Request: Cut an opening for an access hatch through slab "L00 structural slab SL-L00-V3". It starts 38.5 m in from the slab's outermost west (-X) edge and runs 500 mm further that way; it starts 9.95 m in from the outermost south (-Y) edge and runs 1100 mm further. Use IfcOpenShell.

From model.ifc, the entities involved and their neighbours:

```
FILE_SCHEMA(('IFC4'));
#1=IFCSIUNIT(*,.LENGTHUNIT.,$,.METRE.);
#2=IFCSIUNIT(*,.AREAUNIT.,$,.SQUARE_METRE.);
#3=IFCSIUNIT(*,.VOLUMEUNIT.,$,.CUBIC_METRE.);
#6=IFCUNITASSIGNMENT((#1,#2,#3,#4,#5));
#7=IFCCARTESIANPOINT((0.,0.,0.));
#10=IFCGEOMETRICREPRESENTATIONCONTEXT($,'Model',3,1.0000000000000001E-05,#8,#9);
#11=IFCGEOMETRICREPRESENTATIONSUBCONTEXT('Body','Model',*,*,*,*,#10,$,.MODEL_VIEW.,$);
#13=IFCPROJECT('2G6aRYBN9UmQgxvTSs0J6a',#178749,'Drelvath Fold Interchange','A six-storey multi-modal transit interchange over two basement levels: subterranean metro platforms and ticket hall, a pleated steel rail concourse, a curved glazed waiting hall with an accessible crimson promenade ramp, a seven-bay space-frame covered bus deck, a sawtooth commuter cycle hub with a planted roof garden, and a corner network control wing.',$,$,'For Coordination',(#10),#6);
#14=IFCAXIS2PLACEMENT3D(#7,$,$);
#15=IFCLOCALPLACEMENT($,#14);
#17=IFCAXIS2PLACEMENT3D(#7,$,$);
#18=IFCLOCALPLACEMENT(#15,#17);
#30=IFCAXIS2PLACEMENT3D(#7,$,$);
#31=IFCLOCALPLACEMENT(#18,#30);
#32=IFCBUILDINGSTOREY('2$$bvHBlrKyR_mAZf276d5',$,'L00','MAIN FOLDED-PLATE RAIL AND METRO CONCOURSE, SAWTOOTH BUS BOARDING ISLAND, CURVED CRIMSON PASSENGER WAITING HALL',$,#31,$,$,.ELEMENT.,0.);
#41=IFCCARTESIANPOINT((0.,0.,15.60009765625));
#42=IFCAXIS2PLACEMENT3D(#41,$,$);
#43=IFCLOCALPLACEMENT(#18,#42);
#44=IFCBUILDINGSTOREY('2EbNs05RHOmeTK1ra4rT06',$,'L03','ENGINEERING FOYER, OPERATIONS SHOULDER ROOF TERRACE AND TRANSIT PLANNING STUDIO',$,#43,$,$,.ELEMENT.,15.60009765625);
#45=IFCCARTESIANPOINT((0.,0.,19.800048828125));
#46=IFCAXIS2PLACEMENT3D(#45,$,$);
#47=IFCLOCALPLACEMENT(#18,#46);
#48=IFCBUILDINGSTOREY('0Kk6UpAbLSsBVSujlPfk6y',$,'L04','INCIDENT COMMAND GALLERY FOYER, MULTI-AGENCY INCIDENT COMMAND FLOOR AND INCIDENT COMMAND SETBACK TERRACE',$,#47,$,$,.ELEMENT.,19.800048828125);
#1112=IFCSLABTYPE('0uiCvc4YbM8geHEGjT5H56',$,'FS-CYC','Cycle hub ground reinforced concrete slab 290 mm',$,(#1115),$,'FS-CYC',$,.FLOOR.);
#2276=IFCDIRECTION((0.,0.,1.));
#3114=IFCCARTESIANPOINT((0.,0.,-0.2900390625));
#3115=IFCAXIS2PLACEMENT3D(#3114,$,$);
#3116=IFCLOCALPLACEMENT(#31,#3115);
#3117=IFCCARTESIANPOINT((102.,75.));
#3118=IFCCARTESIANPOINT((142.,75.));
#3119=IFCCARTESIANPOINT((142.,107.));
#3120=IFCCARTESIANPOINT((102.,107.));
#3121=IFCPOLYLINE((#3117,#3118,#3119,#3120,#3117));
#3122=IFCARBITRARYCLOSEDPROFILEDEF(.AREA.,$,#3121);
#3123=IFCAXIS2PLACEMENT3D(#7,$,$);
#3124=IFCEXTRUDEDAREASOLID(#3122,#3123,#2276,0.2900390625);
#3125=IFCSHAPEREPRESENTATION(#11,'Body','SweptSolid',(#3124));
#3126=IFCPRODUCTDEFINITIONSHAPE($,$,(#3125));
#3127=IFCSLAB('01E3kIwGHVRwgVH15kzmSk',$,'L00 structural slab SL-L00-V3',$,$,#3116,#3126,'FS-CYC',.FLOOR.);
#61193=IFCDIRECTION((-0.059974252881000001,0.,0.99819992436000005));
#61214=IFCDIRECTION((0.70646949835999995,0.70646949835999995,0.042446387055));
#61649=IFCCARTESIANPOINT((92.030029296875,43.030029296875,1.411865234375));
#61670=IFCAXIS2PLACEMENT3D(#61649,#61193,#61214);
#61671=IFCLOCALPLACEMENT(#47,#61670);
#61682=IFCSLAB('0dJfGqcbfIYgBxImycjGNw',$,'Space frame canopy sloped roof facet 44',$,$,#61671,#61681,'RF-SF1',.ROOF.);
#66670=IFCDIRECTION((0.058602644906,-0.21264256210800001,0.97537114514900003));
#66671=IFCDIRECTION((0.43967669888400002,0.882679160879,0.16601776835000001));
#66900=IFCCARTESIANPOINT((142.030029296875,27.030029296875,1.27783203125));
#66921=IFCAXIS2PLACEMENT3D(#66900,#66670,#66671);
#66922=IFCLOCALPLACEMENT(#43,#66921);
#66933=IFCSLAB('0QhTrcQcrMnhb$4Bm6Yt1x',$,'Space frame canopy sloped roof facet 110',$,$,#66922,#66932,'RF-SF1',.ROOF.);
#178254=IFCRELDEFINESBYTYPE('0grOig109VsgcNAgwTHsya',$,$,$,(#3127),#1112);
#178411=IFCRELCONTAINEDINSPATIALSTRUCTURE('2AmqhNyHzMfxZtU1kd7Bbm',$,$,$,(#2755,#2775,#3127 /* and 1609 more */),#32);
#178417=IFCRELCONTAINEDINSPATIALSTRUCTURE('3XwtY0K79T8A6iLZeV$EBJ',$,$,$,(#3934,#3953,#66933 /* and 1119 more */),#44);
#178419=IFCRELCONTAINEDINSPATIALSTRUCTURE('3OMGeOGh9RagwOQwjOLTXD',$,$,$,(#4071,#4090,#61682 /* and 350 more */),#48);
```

```python
import numpy as np
import ifcopenshell
import ifcopenshell.api.feature
import ifcopenshell.api.geometry
import ifcopenshell.api.root
import ifcopenshell.geom
import ifcopenshell.util.placement
import ifcopenshell.util.representation
import ifcopenshell.util.shape
import ifcopenshell.util.unit

model = ifcopenshell.open("model.ifc")
unit_scale = ifcopenshell.util.unit.calculate_unit_scale(model)
settings = ifcopenshell.geom.settings()


def volume(element):
    """Net volume in cubic metres, openings subtracted."""
    shape = ifcopenshell.geom.create_shape(settings, element)
    return ifcopenshell.util.shape.get_volume(shape.geometry)


slab = model.by_id(3127)
before = volume(slab)

# Extent in the slab's own axes, in metres. The edges named are its -X and -Y sides.
slab_shape = ifcopenshell.geom.create_shape(settings, slab)
vertices = ifcopenshell.util.shape.get_vertices(slab_shape.geometry)
x_min, y_min, bottom = vertices.min(axis=0)
top = vertices[:, 2].max()

opening = ifcopenshell.api.root.create_entity(model, ifc_class="IfcOpeningElement", name="Access hatch opening", predefined_type="OPENING")
context = ifcopenshell.util.representation.get_context(model, "Model", "Body", "MODEL_VIEW")
width, depth = 0.5, 1.1
outline = [(0.0, 0.0), (width, 0.0), (width, depth), (0.0, depth), (0.0, 0.0)]
# Overshoot both faces by 50 mm so the cut is clean.
shape = ifcopenshell.api.geometry.add_slab_representation(
    model, context=context, depth=top - bottom + 0.1, polyline=outline
)
ifcopenshell.api.geometry.assign_representation(model, product=opening, representation=shape)

matrix = ifcopenshell.util.placement.get_local_placement(slab.ObjectPlacement)
matrix[:, 3] = matrix @ np.append(np.array([x_min + 38.5, y_min + 9.95, bottom - 0.05]) / unit_scale, 1.0)
ifcopenshell.api.geometry.edit_object_placement(model, product=opening, matrix=matrix, is_si=False)
ifcopenshell.api.feature.add_feature(model, feature=opening, element=slab)

after = volume(slab)

print(f"slab volume {before:.3f} -> {after:.3f} m3")

model.write("model_edited.ifc")
```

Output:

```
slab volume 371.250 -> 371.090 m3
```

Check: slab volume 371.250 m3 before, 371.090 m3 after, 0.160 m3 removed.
